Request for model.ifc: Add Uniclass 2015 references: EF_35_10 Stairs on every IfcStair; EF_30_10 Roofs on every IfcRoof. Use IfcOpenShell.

First a look at what the model holds.

```python
import ifcopenshell

model = ifcopenshell.open("model.ifc")
print(model.schema)
print("classifications:", [c.Name for c in model.by_type("IfcClassification")])
for ifc_class in ("IfcDoor", "IfcRoof", "IfcStair", "IfcWall", "IfcWindow"):
    print(ifc_class, len(model.by_type(ifc_class)))
```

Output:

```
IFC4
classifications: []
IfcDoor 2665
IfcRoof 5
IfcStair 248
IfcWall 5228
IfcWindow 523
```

```python
import ifcopenshell
import ifcopenshell.api.classification

model = ifcopenshell.open("model.ifc")

system = ifcopenshell.api.classification.add_classification(model, classification="Uniclass 2015")

codes = {
    "IfcStair": ("EF_35_10", "Stairs"),
    "IfcRoof": ("EF_30_10", "Roofs"),
}
for ifc_class, (code, name) in codes.items():
    products = model.by_type(ifc_class)
    ifcopenshell.api.classification.add_reference(
        model, products=products, classification=system, identification=code, name=name
    )
    print(code, len(products))

model.write("model_edited.ifc")
```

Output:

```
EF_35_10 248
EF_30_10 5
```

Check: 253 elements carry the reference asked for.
